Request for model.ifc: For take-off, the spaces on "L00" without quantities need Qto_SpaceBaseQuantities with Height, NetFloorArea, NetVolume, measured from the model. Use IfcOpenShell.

First a look at what the model holds.

```python
import ifcopenshell
import ifcopenshell.util.element
import ifcopenshell.util.unit

model = ifcopenshell.open("model.ifc")
print(model.schema)
for unit_type in ("LENGTHUNIT", "AREAUNIT", "VOLUMEUNIT"):
    print(unit_type, ifcopenshell.util.unit.calculate_unit_scale(model, unit_type))
storey = next(s for s in model.by_type("IfcBuildingStorey") if s.Name == "L00")
spaces = [e for e in ifcopenshell.util.element.get_decomposition(storey) if e.is_a("IfcSpace")]
for e in sorted(spaces, key=lambda e: e.id()):
    print(e.id(), e.is_a(), e.Name, list(ifcopenshell.util.element.get_psets(e, qtos_only=True)), sep=" | ")
```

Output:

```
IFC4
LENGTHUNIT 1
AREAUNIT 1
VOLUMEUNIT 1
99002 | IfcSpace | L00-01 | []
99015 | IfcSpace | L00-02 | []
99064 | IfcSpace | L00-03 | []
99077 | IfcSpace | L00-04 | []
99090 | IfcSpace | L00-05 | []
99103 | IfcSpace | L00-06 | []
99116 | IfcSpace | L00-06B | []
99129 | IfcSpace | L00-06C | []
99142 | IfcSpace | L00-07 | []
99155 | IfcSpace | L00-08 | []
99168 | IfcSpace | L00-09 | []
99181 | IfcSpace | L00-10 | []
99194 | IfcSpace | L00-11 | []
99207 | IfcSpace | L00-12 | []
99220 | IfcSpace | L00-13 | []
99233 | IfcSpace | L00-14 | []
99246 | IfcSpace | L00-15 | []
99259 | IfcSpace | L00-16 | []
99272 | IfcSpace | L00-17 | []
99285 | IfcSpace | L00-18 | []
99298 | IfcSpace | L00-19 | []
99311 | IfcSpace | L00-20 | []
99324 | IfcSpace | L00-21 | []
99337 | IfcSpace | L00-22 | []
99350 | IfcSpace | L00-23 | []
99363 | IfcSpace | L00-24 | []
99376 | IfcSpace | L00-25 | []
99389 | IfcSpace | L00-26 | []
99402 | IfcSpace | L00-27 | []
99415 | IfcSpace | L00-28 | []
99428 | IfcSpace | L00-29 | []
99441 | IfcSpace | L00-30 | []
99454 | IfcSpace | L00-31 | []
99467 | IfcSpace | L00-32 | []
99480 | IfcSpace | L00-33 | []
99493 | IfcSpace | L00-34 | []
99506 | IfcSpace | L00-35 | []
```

```python
import ifcopenshell
import ifcopenshell.api.pset
import ifcopenshell.geom
import ifcopenshell.util.element
import ifcopenshell.util.shape
import ifcopenshell.util.unit

model = ifcopenshell.open("model.ifc")
unit_scale = ifcopenshell.util.unit.calculate_unit_scale(model)
area_scale = ifcopenshell.util.unit.calculate_unit_scale(model, "AREAUNIT")
volume_scale = ifcopenshell.util.unit.calculate_unit_scale(model, "VOLUMEUNIT")
settings = ifcopenshell.geom.settings()

storey = next(s for s in model.by_type("IfcBuildingStorey") if s.Name == "L00")
spaces = [e for e in ifcopenshell.util.element.get_decomposition(storey) if e.is_a("IfcSpace")]

for e in sorted(spaces, key=lambda e: e.id()):
    if ifcopenshell.util.element.get_psets(e, qtos_only=True, should_inherit=False):
        continue
    # Geometry comes back in metres, in the element's own axes.
    shape = ifcopenshell.geom.create_shape(settings, e)
    values = {
        "Height": ifcopenshell.util.shape.get_z(shape.geometry) / unit_scale,
        "NetFloorArea": ifcopenshell.util.shape.get_footprint_area(shape.geometry) / area_scale,
        "NetVolume": ifcopenshell.util.shape.get_volume(shape.geometry) / volume_scale,
    }
    qto = ifcopenshell.api.pset.add_qto(model, product=e, name="Qto_SpaceBaseQuantities")
    ifcopenshell.api.pset.edit_qto(model, qto=qto, properties=values)
    print(e.id(), {k: round(v, 3) for k, v in values.items()})

model.write("model_edited.ifc")
```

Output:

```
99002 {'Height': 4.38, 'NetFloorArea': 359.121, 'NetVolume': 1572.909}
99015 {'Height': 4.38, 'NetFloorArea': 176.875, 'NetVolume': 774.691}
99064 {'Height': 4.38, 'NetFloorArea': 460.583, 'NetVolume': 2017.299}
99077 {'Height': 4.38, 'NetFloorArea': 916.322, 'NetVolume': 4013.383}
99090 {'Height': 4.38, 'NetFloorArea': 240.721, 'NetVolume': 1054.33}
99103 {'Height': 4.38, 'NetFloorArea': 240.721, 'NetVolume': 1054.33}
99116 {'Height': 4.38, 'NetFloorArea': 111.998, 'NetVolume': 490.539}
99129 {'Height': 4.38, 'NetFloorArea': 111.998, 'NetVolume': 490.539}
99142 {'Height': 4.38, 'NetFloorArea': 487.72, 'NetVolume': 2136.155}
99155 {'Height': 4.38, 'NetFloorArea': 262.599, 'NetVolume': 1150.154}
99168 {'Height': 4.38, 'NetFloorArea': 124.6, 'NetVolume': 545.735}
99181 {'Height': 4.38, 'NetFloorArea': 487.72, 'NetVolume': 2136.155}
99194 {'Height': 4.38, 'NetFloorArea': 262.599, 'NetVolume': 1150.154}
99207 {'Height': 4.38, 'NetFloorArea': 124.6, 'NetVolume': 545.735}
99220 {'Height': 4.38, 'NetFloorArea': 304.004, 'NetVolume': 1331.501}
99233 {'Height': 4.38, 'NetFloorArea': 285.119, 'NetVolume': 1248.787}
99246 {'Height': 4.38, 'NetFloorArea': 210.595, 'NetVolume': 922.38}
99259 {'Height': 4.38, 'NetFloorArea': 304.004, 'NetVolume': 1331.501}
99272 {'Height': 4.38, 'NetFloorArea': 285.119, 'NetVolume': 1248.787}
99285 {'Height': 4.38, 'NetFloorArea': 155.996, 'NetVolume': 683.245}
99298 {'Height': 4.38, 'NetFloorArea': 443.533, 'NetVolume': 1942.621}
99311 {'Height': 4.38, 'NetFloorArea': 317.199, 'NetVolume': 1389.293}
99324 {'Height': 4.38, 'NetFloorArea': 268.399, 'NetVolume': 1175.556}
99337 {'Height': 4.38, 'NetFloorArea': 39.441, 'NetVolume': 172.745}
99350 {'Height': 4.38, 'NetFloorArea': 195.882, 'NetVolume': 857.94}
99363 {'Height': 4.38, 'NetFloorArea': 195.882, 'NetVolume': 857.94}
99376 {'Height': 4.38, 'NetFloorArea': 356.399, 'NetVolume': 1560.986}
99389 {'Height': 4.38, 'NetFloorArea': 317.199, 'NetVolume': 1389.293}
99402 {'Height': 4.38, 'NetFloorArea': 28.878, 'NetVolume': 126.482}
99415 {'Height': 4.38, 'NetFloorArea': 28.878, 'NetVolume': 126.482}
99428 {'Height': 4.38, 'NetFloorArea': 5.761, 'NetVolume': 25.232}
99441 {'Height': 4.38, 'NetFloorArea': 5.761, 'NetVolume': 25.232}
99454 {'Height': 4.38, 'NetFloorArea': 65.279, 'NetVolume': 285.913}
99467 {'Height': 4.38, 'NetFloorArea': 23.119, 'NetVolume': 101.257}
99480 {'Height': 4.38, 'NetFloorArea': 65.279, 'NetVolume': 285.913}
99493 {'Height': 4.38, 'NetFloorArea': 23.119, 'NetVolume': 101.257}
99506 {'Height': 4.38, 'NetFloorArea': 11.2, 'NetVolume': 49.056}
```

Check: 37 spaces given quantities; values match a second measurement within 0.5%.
